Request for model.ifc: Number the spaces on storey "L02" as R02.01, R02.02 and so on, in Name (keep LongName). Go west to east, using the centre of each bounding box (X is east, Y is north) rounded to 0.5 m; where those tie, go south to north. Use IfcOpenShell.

First a look at what the model holds.

```python
import ifcopenshell
import ifcopenshell.util.element
import ifcopenshell.util.placement

model = ifcopenshell.open("model.ifc")
print(model.schema)
storey = next(s for s in model.by_type("IfcBuildingStorey") if s.Name == "L02")
spaces = [e for e in ifcopenshell.util.element.get_decomposition(storey) if e.is_a("IfcSpace")]
for e in sorted(spaces, key=lambda e: e.id()):
    origin = ifcopenshell.util.placement.get_local_placement(e.ObjectPlacement)[:3, 3]
    print(e.id(), e.Name, e.LongName, origin.round(2) + 0.0, sep=" | ")
```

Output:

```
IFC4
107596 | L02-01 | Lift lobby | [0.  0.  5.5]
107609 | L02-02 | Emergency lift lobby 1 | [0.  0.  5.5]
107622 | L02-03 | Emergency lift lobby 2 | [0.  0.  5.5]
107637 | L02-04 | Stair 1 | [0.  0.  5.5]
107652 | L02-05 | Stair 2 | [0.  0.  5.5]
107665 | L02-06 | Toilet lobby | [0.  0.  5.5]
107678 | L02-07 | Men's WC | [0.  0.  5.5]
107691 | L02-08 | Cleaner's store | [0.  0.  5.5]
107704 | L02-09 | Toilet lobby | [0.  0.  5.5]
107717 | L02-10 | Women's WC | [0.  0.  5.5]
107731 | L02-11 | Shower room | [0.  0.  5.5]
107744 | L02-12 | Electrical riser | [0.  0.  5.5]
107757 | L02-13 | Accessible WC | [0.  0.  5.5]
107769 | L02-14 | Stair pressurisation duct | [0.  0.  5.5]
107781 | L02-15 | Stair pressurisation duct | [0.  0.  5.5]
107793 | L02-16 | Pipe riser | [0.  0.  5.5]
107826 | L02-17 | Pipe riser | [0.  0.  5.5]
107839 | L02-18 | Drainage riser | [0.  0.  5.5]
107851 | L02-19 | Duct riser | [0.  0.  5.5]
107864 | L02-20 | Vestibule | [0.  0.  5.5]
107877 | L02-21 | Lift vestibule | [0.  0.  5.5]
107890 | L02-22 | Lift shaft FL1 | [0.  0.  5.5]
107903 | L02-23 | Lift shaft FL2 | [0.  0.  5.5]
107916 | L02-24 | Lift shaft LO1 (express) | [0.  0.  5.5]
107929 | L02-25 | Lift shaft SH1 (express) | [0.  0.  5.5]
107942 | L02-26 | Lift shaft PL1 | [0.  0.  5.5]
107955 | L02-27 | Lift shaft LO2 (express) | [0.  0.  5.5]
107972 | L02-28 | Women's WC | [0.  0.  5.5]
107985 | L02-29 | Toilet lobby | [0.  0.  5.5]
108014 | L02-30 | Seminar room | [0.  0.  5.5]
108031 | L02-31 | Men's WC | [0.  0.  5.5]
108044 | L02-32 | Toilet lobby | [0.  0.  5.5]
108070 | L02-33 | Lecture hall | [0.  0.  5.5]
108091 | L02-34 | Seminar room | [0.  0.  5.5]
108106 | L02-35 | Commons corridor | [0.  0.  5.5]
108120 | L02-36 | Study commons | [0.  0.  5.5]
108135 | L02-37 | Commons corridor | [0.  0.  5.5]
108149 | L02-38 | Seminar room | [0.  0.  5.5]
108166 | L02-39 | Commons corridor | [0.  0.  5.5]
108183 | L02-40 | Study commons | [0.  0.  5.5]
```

```python
import ifcopenshell
import ifcopenshell.geom
import ifcopenshell.util.element
import ifcopenshell.util.shape

model = ifcopenshell.open("model.ifc")
settings = ifcopenshell.geom.settings()
settings.set("use-world-coords", True)


def centre(element):
    shape = ifcopenshell.geom.create_shape(settings, element)
    return ifcopenshell.util.shape.get_bbox_centroid(shape.geometry)


storey = next(s for s in model.by_type("IfcBuildingStorey") if s.Name == "L02")
spaces = [e for e in ifcopenshell.util.element.get_decomposition(storey) if e.is_a("IfcSpace")]

# Insertion points can sit at a corner or the storey origin, so sort by the geometry (in metres).
centres = {e: centre(e) for e in spaces}
spaces.sort(key=lambda e: (round(centres[e][0] / 0.5), centres[e][1]))

for i, e in enumerate(spaces, start=1):
    number = f"R02.{i:02d}"
    e.Name = number
    print(e.id(), number)

model.write("model_edited.ifc")
```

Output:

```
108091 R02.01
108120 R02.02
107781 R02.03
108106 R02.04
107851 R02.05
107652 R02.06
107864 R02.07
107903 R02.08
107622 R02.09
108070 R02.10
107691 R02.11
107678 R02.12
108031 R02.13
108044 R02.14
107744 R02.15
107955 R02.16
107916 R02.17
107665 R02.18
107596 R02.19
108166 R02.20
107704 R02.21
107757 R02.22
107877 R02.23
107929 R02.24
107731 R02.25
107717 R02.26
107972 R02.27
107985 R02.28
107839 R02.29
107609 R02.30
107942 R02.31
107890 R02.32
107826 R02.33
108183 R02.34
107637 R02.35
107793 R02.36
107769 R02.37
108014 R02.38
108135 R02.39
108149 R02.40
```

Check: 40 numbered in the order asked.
